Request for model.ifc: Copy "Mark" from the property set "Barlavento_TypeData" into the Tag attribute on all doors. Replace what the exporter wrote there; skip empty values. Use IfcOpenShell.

First a look at what the model holds.

```python
import ifcopenshell
import ifcopenshell.util.element

model = ifcopenshell.open("model.ifc")
print(model.schema)
doors = model.by_type("IfcDoor")
print(len(doors), "doors")
for e in doors[:8]:
    source = ifcopenshell.util.element.get_pset(e, "Barlavento_TypeData", "Mark")
    target = e.Tag
    print(e.id(), repr(source), repr(target), sep=" | ")
```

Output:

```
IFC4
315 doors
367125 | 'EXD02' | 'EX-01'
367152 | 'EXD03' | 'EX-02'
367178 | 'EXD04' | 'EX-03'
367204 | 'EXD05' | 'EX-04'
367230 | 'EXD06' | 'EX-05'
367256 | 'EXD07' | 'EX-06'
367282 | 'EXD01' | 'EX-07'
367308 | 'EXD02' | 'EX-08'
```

```python
import ifcopenshell
import ifcopenshell.util.element

model = ifcopenshell.open("model.ifc")

count = 0
for e in model.by_type("IfcDoor"):
    value = ifcopenshell.util.element.get_pset(e, "Barlavento_TypeData", "Mark")
    current = e.Tag
    if not value or not value.strip() or current == value:
        continue
    e.Tag = value
    count += 1

print(count, "doors updated")

model.write("model_v2.ifc")
```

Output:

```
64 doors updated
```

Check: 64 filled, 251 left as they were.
